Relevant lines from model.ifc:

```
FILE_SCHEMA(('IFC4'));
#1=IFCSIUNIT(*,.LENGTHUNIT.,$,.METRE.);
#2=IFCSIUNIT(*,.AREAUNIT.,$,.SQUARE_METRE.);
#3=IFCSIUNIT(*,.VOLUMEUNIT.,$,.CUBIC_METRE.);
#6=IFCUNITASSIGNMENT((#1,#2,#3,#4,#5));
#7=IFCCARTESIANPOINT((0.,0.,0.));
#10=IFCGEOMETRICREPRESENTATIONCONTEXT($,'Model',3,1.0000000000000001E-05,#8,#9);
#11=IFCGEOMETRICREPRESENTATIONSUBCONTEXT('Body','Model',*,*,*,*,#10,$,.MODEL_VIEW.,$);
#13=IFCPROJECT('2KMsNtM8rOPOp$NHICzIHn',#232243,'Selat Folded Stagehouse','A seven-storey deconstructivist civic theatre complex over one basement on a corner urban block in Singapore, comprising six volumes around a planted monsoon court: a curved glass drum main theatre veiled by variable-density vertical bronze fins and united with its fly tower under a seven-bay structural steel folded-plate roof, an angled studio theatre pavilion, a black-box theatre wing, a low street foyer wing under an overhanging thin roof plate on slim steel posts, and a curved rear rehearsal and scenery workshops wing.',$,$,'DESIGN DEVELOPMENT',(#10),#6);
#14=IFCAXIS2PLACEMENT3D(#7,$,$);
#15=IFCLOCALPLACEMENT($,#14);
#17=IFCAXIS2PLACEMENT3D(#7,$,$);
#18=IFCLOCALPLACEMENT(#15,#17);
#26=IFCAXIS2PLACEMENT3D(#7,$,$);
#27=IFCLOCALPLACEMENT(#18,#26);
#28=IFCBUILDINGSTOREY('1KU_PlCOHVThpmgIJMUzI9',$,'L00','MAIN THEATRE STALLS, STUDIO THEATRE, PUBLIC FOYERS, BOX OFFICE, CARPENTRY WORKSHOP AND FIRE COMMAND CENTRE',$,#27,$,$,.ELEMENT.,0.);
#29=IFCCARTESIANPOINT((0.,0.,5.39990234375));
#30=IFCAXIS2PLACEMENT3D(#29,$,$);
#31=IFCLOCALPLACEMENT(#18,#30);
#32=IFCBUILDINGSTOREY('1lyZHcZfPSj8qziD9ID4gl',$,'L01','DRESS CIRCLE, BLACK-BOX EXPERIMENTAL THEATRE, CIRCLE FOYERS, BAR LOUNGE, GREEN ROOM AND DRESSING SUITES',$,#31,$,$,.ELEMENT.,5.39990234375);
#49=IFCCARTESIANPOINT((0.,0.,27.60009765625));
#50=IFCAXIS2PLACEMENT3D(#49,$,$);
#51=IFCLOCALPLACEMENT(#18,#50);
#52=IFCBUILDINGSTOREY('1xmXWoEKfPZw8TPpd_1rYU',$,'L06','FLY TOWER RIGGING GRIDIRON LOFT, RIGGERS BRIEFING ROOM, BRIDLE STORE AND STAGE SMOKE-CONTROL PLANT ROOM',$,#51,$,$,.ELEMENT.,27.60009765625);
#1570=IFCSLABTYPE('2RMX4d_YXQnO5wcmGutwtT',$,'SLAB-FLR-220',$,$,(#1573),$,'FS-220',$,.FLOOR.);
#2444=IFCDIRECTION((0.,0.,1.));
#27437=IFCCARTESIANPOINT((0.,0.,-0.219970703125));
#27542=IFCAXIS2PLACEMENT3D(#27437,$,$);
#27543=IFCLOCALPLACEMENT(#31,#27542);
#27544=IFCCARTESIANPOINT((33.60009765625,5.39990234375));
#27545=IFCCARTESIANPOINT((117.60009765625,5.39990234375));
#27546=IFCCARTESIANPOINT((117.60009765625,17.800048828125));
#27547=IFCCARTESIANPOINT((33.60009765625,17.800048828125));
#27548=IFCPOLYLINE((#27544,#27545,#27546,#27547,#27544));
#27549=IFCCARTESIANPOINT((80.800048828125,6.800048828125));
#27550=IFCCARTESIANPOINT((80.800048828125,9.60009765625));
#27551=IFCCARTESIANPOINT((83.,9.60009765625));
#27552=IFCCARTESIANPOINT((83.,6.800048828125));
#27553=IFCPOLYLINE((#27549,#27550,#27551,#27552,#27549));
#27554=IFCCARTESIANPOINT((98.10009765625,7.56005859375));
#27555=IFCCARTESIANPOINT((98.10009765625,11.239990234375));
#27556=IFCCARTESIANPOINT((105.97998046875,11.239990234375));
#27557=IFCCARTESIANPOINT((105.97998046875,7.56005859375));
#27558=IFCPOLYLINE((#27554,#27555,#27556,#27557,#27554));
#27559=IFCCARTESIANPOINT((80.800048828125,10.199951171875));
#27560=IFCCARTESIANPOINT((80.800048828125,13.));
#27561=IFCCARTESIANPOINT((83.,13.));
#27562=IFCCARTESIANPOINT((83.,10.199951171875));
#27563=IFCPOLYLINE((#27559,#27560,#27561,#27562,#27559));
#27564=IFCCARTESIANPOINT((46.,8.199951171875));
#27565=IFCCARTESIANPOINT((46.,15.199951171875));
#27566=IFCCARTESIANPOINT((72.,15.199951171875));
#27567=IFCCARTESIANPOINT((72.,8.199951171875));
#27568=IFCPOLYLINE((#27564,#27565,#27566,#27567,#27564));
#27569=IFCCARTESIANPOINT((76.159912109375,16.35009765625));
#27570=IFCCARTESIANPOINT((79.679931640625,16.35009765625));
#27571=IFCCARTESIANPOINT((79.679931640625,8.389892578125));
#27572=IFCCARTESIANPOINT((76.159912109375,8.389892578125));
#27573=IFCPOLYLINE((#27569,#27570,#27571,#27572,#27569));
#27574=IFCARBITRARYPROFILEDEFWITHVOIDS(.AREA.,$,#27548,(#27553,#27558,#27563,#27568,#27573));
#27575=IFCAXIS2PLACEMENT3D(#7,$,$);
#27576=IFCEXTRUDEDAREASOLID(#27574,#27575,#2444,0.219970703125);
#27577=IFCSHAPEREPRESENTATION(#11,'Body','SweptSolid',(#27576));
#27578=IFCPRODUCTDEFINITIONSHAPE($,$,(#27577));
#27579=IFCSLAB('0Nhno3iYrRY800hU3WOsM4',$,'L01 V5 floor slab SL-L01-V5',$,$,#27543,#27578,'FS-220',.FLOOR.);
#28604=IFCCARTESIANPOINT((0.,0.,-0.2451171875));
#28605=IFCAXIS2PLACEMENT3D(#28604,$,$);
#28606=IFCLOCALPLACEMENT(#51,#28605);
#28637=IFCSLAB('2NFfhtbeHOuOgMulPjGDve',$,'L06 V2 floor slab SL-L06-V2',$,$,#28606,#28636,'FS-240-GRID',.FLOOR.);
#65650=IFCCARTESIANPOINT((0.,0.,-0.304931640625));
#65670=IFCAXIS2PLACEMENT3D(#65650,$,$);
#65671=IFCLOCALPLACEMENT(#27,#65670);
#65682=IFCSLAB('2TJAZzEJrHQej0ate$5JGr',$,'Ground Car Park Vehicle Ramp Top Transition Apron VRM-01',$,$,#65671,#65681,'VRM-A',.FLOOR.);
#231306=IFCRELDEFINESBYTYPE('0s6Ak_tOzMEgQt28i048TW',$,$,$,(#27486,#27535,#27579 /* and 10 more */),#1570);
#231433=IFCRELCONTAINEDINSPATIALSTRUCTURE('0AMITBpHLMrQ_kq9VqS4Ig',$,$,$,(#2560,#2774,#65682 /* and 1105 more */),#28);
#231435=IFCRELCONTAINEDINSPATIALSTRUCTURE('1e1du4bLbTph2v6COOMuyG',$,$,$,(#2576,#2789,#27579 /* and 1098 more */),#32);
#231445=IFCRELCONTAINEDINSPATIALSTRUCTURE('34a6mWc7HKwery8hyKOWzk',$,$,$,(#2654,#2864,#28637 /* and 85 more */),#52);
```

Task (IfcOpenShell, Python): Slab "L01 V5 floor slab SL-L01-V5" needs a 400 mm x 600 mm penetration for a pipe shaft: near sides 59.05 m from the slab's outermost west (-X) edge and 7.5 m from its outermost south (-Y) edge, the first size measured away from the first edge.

```python
import numpy as np
import ifcopenshell
import ifcopenshell.api.feature
import ifcopenshell.api.geometry
import ifcopenshell.api.root
import ifcopenshell.geom
import ifcopenshell.util.placement
import ifcopenshell.util.representation
import ifcopenshell.util.shape
import ifcopenshell.util.unit

model = ifcopenshell.open("model.ifc")
unit_scale = ifcopenshell.util.unit.calculate_unit_scale(model)
settings = ifcopenshell.geom.settings()


def volume(element):
    """Net volume in cubic metres, openings subtracted."""
    shape = ifcopenshell.geom.create_shape(settings, element)
    return ifcopenshell.util.shape.get_volume(shape.geometry)


slab = model.by_guid("0Nhno3iYrRY800hU3WOsM4")
before = volume(slab)

# Extent in the slab's own axes, in metres. The edges named are its -X and -Y sides.
slab_shape = ifcopenshell.geom.create_shape(settings, slab)
vertices = ifcopenshell.util.shape.get_vertices(slab_shape.geometry)
x_min, y_min, bottom = vertices.min(axis=0)
top = vertices[:, 2].max()

opening = ifcopenshell.api.root.create_entity(model, ifc_class="IfcOpeningElement", name="Pipe shaft opening", predefined_type="OPENING")
context = ifcopenshell.util.representation.get_context(model, "Model", "Body", "MODEL_VIEW")
width, depth = 0.4, 0.6
outline = [(0.0, 0.0), (width, 0.0), (width, depth), (0.0, depth), (0.0, 0.0)]
# Overshoot both faces by 50 mm so the cut is clean.
shape = ifcopenshell.api.geometry.add_slab_representation(
    model, context=context, depth=top - bottom + 0.1, polyline=outline
)
ifcopenshell.api.geometry.assign_representation(model, product=opening, representation=shape)

matrix = ifcopenshell.util.placement.get_local_placement(slab.ObjectPlacement)
matrix[:, 3] = matrix @ np.append(np.array([x_min + 59.05, y_min + 7.5, bottom - 0.05]) / unit_scale, 1.0)
ifcopenshell.api.geometry.edit_object_placement(model, product=opening, matrix=matrix, is_si=False)
ifcopenshell.api.feature.add_feature(model, feature=opening, element=slab)

after = volume(slab)

print(f"slab volume {before:.3f} -> {after:.3f} m3")

model.write("model_updated.ifc")
```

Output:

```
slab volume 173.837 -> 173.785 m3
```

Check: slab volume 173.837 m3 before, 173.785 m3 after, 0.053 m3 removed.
